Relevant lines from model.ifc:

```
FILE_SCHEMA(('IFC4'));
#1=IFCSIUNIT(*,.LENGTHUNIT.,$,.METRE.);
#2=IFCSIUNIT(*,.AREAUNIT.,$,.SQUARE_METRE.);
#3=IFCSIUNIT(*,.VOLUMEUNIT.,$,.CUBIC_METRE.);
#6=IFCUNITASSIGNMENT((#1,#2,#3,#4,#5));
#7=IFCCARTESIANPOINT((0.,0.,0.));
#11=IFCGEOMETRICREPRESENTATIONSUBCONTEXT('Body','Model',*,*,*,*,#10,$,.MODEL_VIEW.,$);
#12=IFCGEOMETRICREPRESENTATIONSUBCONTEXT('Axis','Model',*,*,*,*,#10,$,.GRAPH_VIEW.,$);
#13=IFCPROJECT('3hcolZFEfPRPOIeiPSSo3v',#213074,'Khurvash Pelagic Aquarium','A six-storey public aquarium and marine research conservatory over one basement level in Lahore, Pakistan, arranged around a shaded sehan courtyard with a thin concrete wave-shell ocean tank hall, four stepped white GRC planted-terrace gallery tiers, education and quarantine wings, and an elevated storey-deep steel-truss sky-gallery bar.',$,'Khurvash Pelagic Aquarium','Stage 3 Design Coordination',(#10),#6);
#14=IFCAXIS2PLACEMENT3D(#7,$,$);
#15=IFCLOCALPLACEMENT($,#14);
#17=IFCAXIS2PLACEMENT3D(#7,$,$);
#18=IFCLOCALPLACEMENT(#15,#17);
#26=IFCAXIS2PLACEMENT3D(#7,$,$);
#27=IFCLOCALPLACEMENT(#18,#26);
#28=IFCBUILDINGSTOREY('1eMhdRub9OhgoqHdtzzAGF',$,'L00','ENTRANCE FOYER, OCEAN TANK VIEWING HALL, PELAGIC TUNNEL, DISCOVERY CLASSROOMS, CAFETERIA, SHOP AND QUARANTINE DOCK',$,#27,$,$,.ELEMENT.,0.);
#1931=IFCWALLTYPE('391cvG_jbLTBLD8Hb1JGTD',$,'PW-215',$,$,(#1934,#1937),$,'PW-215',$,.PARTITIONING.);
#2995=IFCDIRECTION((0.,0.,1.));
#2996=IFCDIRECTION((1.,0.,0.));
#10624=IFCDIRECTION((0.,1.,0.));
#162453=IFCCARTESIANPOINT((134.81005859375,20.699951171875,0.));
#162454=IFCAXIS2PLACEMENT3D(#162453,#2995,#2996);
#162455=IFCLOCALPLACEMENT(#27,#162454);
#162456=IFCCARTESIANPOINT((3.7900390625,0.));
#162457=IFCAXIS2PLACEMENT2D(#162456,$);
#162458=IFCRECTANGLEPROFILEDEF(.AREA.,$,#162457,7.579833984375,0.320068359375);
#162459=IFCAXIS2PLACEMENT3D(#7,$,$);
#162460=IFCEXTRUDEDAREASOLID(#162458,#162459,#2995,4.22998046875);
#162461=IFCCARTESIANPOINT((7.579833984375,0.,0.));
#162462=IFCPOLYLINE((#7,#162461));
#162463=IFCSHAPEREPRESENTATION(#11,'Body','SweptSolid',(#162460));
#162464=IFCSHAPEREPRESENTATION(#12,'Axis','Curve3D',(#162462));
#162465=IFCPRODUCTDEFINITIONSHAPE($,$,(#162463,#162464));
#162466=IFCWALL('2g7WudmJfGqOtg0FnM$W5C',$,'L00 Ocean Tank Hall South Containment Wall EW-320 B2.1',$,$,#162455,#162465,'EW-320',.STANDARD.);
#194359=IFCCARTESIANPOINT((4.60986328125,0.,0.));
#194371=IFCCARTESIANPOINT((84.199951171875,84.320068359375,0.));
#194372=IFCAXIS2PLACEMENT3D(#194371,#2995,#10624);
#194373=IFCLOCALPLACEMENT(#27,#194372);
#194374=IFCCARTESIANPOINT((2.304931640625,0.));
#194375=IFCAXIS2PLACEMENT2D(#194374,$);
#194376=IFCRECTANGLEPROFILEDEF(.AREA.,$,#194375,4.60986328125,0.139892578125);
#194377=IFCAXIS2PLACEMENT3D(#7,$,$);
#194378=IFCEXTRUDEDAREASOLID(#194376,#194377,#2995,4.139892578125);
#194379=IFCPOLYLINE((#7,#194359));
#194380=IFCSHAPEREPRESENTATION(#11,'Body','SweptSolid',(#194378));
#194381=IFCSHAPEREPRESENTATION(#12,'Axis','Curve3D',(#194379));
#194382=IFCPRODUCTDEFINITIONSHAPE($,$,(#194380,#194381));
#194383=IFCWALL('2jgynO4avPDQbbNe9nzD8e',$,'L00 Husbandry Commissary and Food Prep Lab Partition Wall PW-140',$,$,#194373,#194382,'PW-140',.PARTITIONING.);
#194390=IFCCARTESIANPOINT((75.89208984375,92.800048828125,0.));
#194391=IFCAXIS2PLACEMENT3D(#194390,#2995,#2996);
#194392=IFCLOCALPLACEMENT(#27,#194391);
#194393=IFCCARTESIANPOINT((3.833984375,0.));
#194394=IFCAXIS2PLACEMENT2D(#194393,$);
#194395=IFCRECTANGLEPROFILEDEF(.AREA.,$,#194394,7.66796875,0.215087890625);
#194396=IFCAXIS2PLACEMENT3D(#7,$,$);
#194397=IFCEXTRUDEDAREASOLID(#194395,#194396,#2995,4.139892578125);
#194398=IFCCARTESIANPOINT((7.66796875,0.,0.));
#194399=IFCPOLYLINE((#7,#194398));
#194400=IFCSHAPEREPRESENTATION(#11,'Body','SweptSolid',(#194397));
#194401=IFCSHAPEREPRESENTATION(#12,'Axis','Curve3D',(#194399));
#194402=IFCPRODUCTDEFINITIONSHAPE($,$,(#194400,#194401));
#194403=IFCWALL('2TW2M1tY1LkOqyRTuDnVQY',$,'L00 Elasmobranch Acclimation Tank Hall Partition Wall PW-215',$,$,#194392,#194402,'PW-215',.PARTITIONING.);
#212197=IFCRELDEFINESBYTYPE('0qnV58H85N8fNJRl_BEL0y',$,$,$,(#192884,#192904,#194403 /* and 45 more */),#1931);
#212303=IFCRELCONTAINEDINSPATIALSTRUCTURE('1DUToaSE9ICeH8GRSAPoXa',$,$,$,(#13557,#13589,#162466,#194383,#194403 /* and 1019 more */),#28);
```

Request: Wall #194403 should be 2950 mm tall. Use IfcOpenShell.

```python
import ifcopenshell
import ifcopenshell.geom
import ifcopenshell.util.representation
import ifcopenshell.util.shape
import ifcopenshell.util.unit

model = ifcopenshell.open("model.ifc")
unit_scale = ifcopenshell.util.unit.calculate_unit_scale(model)
settings = ifcopenshell.geom.settings()


def volume(element):
    """Net volume in cubic metres, openings subtracted."""
    shape = ifcopenshell.geom.create_shape(settings, element)
    return ifcopenshell.util.shape.get_volume(shape.geometry)


wall = model.by_guid("2TW2M1tY1LkOqyRTuDnVQY")
before = volume(wall)

body = ifcopenshell.util.representation.get_representation(wall, "Model", "Body")
solid = body.Items[0]
old_height = solid.Depth
solid.Depth = 2.95 / unit_scale
after = volume(wall)

print(f"height {old_height:g} -> {solid.Depth:g}, volume {before:.3f} -> {after:.3f} m3")

model.write("model_updated.ifc")
```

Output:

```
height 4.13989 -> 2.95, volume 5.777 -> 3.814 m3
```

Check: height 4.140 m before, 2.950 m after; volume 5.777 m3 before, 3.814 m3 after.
